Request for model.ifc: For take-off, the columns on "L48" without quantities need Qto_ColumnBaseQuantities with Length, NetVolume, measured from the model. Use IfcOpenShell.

First a look at what the model holds.

```python
import ifcopenshell
import ifcopenshell.util.element
import ifcopenshell.util.unit

model = ifcopenshell.open("model.ifc")
print(model.schema)
for unit_type in ("LENGTHUNIT", "AREAUNIT", "VOLUMEUNIT"):
    print(unit_type, ifcopenshell.util.unit.calculate_unit_scale(model, unit_type))
storey = next(s for s in model.by_type("IfcBuildingStorey") if s.Name == "L48")
columns = [e for e in ifcopenshell.util.element.get_decomposition(storey) if e.is_a("IfcColumn")]
for e in sorted(columns, key=lambda e: e.id()):
    print(e.id(), e.is_a(), e.Name, list(ifcopenshell.util.element.get_psets(e, qtos_only=True)), sep=" | ")
```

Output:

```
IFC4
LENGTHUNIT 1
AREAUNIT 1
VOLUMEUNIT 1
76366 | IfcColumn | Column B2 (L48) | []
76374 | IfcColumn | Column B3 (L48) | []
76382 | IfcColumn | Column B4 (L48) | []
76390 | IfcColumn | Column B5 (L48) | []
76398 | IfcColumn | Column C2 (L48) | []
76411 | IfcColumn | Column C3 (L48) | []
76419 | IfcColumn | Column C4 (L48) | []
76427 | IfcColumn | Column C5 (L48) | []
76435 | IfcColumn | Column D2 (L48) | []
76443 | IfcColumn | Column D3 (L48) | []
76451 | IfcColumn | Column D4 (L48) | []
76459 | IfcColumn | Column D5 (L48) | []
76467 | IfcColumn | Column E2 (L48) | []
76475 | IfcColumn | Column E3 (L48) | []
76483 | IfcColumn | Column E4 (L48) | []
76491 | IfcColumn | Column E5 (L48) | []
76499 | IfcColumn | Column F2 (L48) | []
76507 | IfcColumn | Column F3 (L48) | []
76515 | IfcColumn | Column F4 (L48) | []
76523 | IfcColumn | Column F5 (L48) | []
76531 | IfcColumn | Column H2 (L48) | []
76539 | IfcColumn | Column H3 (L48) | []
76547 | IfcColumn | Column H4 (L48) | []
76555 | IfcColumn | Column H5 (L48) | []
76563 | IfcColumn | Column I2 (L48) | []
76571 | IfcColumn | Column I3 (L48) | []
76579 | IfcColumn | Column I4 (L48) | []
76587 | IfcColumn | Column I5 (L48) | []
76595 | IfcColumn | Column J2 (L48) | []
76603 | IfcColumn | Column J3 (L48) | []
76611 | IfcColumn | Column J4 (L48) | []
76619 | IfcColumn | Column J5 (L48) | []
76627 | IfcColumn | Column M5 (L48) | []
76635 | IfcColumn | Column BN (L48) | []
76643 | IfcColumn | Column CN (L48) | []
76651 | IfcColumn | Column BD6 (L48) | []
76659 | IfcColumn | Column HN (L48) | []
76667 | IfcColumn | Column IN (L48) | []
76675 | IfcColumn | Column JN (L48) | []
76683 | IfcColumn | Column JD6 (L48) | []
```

```python
import ifcopenshell
import ifcopenshell.api.pset
import ifcopenshell.geom
import ifcopenshell.util.element
import ifcopenshell.util.shape
import ifcopenshell.util.unit

model = ifcopenshell.open("model.ifc")
unit_scale = ifcopenshell.util.unit.calculate_unit_scale(model)
volume_scale = ifcopenshell.util.unit.calculate_unit_scale(model, "VOLUMEUNIT")
settings = ifcopenshell.geom.settings()

storey = next(s for s in model.by_type("IfcBuildingStorey") if s.Name == "L48")
columns = [e for e in ifcopenshell.util.element.get_decomposition(storey) if e.is_a("IfcColumn")]

for e in sorted(columns, key=lambda e: e.id()):
    if ifcopenshell.util.element.get_psets(e, qtos_only=True, should_inherit=False):
        continue
    # Geometry comes back in metres, in the element's own axes.
    shape = ifcopenshell.geom.create_shape(settings, e)
    values = {
        "Length": ifcopenshell.util.shape.get_z(shape.geometry) / unit_scale,
        "NetVolume": ifcopenshell.util.shape.get_volume(shape.geometry) / volume_scale,
    }
    qto = ifcopenshell.api.pset.add_qto(model, product=e, name="Qto_ColumnBaseQuantities")
    ifcopenshell.api.pset.edit_qto(model, qto=qto, properties=values)
    print(e.id(), {k: round(v, 3) for k, v in values.items()})

model.write("model-out.ifc")
```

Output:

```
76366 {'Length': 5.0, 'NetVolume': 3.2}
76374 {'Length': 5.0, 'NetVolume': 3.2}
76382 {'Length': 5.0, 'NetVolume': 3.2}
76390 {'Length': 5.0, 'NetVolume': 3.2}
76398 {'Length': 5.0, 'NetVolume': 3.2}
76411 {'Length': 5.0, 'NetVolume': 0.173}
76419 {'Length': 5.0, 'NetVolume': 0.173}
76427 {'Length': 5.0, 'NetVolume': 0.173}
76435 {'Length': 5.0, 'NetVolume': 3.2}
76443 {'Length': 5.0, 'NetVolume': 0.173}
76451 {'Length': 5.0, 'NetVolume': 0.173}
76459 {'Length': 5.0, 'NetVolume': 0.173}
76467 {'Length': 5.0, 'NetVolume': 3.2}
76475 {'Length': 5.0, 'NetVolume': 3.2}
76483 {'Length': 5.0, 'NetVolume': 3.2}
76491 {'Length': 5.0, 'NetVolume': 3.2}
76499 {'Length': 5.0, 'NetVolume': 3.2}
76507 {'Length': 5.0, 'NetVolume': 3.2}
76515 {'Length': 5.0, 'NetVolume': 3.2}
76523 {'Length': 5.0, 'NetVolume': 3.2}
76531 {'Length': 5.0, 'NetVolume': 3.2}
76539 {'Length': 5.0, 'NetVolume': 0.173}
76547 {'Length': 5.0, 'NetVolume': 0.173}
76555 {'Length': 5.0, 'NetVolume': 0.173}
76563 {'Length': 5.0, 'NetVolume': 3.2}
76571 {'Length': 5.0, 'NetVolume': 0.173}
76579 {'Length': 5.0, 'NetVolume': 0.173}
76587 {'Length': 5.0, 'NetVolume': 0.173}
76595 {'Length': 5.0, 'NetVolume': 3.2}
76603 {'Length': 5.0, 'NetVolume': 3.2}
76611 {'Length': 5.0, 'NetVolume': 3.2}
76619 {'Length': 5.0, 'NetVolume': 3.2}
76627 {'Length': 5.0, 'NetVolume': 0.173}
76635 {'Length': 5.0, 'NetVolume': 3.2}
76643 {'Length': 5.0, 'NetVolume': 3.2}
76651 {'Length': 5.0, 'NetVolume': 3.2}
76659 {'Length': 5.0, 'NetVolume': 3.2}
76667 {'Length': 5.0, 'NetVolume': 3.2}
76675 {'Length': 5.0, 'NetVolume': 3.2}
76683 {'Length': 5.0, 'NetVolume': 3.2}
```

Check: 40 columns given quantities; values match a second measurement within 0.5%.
